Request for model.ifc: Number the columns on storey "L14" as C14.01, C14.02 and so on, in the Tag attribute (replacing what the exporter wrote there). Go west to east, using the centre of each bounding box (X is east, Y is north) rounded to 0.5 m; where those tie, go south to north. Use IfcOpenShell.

First a look at what the model holds.

```python
import ifcopenshell
import ifcopenshell.util.element
import ifcopenshell.util.placement

model = ifcopenshell.open("model.ifc")
print(model.schema)
storey = next(s for s in model.by_type("IfcBuildingStorey") if s.Name == "L14")
columns = [e for e in ifcopenshell.util.element.get_decomposition(storey) if e.is_a("IfcColumn")]
for e in sorted(columns, key=lambda e: e.id()):
    origin = ifcopenshell.util.placement.get_local_placement(e.ObjectPlacement)[:3, 3]
    print(e.id(), e.Tag, e.Name, origin.round(2) + 0.0, sep=" | ")
```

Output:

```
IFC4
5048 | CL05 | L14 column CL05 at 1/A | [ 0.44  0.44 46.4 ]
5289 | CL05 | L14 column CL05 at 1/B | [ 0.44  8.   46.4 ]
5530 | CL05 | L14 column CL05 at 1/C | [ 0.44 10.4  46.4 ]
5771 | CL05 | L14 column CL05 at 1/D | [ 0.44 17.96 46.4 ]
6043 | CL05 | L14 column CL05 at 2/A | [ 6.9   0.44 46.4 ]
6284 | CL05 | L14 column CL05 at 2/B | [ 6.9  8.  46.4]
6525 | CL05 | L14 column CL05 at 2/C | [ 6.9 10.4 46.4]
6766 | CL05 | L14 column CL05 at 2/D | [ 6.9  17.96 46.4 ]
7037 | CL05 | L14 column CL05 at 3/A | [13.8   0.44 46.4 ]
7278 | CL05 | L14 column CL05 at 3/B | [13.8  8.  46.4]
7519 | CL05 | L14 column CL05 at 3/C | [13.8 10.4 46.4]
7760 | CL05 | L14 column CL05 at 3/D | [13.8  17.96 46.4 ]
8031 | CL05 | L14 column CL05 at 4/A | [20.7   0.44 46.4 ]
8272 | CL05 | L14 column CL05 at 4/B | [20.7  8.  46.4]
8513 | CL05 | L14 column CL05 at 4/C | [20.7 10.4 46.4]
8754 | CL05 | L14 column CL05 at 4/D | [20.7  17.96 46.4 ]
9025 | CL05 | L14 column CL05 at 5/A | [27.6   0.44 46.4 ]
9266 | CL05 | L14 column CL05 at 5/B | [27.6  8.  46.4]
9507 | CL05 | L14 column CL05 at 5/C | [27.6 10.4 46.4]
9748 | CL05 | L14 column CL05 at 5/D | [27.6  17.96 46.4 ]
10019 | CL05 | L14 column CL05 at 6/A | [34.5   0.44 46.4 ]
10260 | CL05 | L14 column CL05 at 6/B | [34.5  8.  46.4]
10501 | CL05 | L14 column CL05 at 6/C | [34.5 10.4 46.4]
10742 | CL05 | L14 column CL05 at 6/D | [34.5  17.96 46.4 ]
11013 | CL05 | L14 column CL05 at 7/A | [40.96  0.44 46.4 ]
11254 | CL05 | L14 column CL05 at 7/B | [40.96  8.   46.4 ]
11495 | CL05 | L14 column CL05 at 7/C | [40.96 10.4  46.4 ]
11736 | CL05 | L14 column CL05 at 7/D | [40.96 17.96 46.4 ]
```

```python
import ifcopenshell
import ifcopenshell.geom
import ifcopenshell.util.element
import ifcopenshell.util.shape

model = ifcopenshell.open("model.ifc")
settings = ifcopenshell.geom.settings()
settings.set("use-world-coords", True)


def centre(element):
    shape = ifcopenshell.geom.create_shape(settings, element)
    return ifcopenshell.util.shape.get_bbox_centroid(shape.geometry)


storey = next(s for s in model.by_type("IfcBuildingStorey") if s.Name == "L14")
columns = [e for e in ifcopenshell.util.element.get_decomposition(storey) if e.is_a("IfcColumn")]

# Insertion points can sit at a corner or the storey origin, so sort by the geometry (in metres).
centres = {e: centre(e) for e in columns}
columns.sort(key=lambda e: (round(centres[e][0] / 0.5), centres[e][1]))

for i, e in enumerate(columns, start=1):
    number = f"C14.{i:02d}"
    e.Tag = number
    print(e.id(), number)

model.write("model-out.ifc")
```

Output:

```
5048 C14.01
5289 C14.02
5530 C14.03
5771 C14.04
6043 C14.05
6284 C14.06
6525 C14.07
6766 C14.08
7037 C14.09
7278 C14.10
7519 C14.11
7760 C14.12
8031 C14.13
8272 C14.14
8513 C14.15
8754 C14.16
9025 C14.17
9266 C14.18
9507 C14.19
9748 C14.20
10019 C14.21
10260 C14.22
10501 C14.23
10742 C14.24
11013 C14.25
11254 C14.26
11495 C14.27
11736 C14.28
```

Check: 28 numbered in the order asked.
